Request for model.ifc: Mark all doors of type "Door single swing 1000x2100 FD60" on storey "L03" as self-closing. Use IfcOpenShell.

First a look at what the model holds.

```python
import ifcopenshell
import ifcopenshell.util.element

model = ifcopenshell.open("model.ifc")
print(model.schema)
storey = next(s for s in model.by_type("IfcBuildingStorey") if s.Name == "L03")
doors = [e for e in ifcopenshell.util.element.get_decomposition(storey) if e.is_a("IfcDoor")]
seen = {}
for e in doors:
    element_type = ifcopenshell.util.element.get_type(e)
    key = (element_type.Name if element_type != e and element_type else None, ifcopenshell.util.element.get_pset(e, "Pset_DoorCommon", "SelfClosing"))
    seen[key] = seen.get(key, 0) + 1
for (name, value), count in sorted(seen.items(), key=str):
    print(count, "x", name, "|", value)
```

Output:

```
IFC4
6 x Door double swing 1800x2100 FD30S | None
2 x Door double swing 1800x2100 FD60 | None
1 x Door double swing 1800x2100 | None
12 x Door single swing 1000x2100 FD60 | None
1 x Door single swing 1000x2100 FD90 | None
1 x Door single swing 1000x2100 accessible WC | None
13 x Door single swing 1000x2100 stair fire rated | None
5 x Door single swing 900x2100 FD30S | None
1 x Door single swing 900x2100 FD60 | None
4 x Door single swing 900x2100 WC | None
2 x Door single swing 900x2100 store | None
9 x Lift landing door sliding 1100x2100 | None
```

```python
import ifcopenshell
import ifcopenshell.api.pset
import ifcopenshell.util.element

model = ifcopenshell.open("model.ifc")

storey = next(s for s in model.by_type("IfcBuildingStorey") if s.Name == "L03")
doors = [e for e in ifcopenshell.util.element.get_decomposition(storey) if e.is_a("IfcDoor")]

count = 0
for e in doors:
    element_type = ifcopenshell.util.element.get_type(e)
    if element_type in (None, e) or element_type.Name != "Door single swing 1000x2100 FD60":
        continue
    # add_pset returns the element's existing set when there is one.
    pset = ifcopenshell.api.pset.add_pset(model, product=e, name="Pset_DoorCommon")
    ifcopenshell.api.pset.edit_pset(model, pset=pset, properties={"SelfClosing": True})
    count += 1

print(count, "doors updated")

model.write("model_edited.ifc")
```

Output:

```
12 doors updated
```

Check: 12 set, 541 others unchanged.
